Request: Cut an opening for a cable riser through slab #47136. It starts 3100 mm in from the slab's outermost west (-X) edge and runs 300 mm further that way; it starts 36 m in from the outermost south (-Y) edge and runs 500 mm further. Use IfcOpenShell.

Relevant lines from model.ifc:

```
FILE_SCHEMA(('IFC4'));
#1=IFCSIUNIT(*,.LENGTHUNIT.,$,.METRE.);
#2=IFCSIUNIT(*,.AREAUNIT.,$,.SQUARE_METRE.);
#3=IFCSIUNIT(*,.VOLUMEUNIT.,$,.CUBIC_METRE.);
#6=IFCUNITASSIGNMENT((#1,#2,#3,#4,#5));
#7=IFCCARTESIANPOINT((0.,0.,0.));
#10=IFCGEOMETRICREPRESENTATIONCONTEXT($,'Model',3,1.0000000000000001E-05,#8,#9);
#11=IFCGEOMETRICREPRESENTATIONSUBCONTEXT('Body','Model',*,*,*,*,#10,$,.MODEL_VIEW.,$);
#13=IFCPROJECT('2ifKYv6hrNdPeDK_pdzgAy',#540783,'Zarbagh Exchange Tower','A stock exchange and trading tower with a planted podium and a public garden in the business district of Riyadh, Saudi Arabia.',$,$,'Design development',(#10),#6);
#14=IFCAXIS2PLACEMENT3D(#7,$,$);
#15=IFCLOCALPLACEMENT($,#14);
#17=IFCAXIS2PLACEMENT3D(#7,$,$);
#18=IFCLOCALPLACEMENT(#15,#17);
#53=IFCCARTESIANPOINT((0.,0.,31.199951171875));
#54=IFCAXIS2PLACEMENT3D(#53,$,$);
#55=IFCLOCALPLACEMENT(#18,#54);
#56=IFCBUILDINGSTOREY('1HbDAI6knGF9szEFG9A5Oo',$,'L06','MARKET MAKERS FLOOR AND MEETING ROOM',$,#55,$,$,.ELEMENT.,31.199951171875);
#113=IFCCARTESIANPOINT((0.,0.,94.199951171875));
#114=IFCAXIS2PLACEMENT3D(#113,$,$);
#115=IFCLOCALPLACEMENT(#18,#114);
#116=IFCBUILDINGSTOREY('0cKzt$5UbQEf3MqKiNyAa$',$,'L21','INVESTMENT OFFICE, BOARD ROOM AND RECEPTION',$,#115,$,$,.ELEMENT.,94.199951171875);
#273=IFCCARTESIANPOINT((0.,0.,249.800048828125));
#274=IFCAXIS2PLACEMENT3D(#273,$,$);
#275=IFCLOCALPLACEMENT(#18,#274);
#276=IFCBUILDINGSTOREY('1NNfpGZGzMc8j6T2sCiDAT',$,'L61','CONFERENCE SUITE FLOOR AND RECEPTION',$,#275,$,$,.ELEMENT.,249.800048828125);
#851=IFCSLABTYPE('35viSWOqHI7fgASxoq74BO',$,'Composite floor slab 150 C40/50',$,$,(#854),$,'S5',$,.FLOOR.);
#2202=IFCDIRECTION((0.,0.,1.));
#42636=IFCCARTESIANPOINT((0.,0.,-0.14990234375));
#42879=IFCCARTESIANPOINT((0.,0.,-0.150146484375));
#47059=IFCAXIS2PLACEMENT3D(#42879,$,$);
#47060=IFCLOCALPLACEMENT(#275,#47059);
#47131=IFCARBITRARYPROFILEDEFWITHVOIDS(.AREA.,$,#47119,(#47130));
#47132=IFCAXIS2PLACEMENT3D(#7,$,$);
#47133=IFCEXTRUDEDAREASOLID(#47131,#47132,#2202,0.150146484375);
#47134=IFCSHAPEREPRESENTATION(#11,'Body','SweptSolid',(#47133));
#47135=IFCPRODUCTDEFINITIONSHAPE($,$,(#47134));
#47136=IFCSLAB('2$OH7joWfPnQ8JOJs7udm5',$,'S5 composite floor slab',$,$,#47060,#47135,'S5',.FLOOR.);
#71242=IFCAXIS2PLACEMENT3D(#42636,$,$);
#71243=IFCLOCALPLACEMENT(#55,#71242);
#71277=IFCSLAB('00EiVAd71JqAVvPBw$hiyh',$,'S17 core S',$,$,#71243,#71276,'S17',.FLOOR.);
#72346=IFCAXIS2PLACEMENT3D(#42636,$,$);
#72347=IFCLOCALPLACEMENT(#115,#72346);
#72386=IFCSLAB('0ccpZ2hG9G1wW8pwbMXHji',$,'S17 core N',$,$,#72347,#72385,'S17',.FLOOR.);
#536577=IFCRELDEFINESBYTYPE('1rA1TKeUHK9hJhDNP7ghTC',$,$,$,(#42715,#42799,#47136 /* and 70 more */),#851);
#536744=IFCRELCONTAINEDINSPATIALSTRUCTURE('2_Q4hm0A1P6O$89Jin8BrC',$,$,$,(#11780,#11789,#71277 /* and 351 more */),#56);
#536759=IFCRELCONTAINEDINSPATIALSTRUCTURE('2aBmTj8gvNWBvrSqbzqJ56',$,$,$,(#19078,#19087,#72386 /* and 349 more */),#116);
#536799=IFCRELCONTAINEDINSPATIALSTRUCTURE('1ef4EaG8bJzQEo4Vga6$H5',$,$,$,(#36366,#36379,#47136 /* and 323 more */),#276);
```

```python
import numpy as np
import ifcopenshell
import ifcopenshell.api.feature
import ifcopenshell.api.geometry
import ifcopenshell.api.root
import ifcopenshell.geom
import ifcopenshell.util.placement
import ifcopenshell.util.representation
import ifcopenshell.util.shape
import ifcopenshell.util.unit

model = ifcopenshell.open("model.ifc")
unit_scale = ifcopenshell.util.unit.calculate_unit_scale(model)
settings = ifcopenshell.geom.settings()


def volume(element):
    """Net volume in cubic metres, openings subtracted."""
    shape = ifcopenshell.geom.create_shape(settings, element)
    return ifcopenshell.util.shape.get_volume(shape.geometry)


slab = model.by_guid("2$OH7joWfPnQ8JOJs7udm5")
before = volume(slab)

# Extent in the slab's own axes, in metres. The edges named are its -X and -Y sides.
slab_shape = ifcopenshell.geom.create_shape(settings, slab)
vertices = ifcopenshell.util.shape.get_vertices(slab_shape.geometry)
x_min, y_min, bottom = vertices.min(axis=0)
top = vertices[:, 2].max()

opening = ifcopenshell.api.root.create_entity(model, ifc_class="IfcOpeningElement", name="Cable riser opening", predefined_type="OPENING")
context = ifcopenshell.util.representation.get_context(model, "Model", "Body", "MODEL_VIEW")
width, depth = 0.3, 0.5
outline = [(0.0, 0.0), (width, 0.0), (width, depth), (0.0, depth), (0.0, 0.0)]
# Overshoot both faces by 50 mm so the cut is clean.
shape = ifcopenshell.api.geometry.add_slab_representation(
    model, context=context, depth=top - bottom + 0.1, polyline=outline
)
ifcopenshell.api.geometry.assign_representation(model, product=opening, representation=shape)

matrix = ifcopenshell.util.placement.get_local_placement(slab.ObjectPlacement)
matrix[:, 3] = matrix @ np.append(np.array([x_min + 3.1, y_min + 36, bottom - 0.05]) / unit_scale, 1.0)
ifcopenshell.api.geometry.edit_object_placement(model, product=opening, matrix=matrix, is_si=False)
ifcopenshell.api.feature.add_feature(model, feature=opening, element=slab)

after = volume(slab)

print(f"slab volume {before:.3f} -> {after:.3f} m3")

model.write("model_updated.ifc")
```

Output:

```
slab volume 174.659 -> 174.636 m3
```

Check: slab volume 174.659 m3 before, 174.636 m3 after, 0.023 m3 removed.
